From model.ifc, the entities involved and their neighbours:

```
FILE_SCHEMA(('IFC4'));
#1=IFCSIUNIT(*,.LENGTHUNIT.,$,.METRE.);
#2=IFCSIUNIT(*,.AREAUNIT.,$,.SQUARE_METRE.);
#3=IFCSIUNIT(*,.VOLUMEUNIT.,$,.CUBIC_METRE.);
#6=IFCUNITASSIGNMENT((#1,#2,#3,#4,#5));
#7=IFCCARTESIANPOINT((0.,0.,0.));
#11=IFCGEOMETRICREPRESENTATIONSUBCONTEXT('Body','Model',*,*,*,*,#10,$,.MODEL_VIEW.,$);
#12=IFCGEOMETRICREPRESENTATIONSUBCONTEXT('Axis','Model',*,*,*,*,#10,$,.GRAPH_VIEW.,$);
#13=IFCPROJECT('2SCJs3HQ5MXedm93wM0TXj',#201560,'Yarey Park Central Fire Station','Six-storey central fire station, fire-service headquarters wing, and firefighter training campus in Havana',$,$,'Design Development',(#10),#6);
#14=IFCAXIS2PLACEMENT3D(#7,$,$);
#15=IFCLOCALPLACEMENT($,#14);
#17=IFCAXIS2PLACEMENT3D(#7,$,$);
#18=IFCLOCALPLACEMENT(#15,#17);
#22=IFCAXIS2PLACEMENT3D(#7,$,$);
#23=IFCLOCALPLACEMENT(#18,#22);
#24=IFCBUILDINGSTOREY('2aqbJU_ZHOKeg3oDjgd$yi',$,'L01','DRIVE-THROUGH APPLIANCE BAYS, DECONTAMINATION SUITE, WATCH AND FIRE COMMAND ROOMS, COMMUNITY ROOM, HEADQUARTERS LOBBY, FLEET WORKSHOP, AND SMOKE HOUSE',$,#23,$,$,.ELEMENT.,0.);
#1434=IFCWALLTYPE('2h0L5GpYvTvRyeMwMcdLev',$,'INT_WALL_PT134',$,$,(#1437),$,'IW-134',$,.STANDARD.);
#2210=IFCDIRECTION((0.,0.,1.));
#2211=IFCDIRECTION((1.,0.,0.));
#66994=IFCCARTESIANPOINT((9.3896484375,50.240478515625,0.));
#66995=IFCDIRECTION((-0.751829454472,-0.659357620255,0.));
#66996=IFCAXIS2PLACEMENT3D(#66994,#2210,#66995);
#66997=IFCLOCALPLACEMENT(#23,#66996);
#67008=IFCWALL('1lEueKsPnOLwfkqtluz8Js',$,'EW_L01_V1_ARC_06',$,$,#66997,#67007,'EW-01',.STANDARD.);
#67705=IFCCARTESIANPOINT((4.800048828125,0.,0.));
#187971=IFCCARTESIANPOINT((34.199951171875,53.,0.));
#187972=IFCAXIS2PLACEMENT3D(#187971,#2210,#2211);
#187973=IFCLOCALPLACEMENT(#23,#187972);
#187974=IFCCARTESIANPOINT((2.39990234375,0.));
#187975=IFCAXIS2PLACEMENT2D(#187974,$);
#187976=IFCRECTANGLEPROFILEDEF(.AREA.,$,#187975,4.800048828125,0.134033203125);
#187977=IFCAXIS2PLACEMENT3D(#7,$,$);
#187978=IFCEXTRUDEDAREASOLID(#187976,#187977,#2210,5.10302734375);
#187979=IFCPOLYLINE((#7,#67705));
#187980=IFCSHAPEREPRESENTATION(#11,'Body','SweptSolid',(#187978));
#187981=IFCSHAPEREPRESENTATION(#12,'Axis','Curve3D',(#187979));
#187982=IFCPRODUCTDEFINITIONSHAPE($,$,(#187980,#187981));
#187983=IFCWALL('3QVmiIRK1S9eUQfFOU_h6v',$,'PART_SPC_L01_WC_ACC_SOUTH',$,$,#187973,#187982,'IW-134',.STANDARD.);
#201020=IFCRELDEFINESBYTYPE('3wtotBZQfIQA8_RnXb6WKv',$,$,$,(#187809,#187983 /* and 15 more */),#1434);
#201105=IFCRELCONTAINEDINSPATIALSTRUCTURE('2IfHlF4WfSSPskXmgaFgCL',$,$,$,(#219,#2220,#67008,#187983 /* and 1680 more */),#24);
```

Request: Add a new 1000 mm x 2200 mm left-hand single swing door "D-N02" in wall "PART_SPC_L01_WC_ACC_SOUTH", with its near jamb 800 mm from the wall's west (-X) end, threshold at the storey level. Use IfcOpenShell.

```python
import numpy as np
import ifcopenshell
import ifcopenshell.api.feature
import ifcopenshell.api.geometry
import ifcopenshell.api.root
import ifcopenshell.api.spatial
import ifcopenshell.geom
import ifcopenshell.util.element
import ifcopenshell.util.placement
import ifcopenshell.util.representation
import ifcopenshell.util.shape
import ifcopenshell.util.unit

model = ifcopenshell.open("model.ifc")
unit_scale = ifcopenshell.util.unit.calculate_unit_scale(model)
settings = ifcopenshell.geom.settings()


def volume(element):
    """Net volume in cubic metres, openings subtracted."""
    shape = ifcopenshell.geom.create_shape(settings, element)
    return ifcopenshell.util.shape.get_volume(shape.geometry)


wall = model.by_guid("3QVmiIRK1S9eUQfFOU_h6v")
storey = ifcopenshell.util.element.get_container(wall, ifc_class="IfcBuildingStorey")
context = ifcopenshell.util.representation.get_context(model, "Model", "Body", "MODEL_VIEW")
before = volume(wall)

width, height, from_end, sill = 1, 2.2, 0.8, 0.0  # metres

# The wall runs along its own X axis, and the end named is its -X end.
wall_shape = ifcopenshell.geom.create_shape(settings, wall)
x, y, z = ifcopenshell.util.shape.get_vertices(wall_shape.geometry).T
start = x.min() + from_end
face, thickness = float(y.min()), float(y.max() - y.min())
wall_matrix = ifcopenshell.util.placement.get_local_placement(wall.ObjectPlacement)
level = ifcopenshell.util.placement.get_local_placement(storey.ObjectPlacement)[2, 3]


def in_wall(x, y):
    """Placement at x, y metres in the wall's axes, at sill height."""
    matrix = wall_matrix.copy()
    matrix[:, 3] = wall_matrix @ np.array([x / unit_scale, y / unit_scale, 0.0, 1.0])
    matrix[2, 3] = level + sill / unit_scale
    return matrix


# Opening: a box that overshoots both wall faces by 50 mm.
opening = ifcopenshell.api.root.create_entity(model, ifc_class="IfcOpeningElement", predefined_type="OPENING")
box = ifcopenshell.api.geometry.add_wall_representation(
    model, context=context, length=width, height=height, thickness=thickness + 0.1
)
ifcopenshell.api.geometry.assign_representation(model, product=opening, representation=box)
ifcopenshell.api.geometry.edit_object_placement(model, product=opening, matrix=in_wall(start, face - 0.05), is_si=False)
ifcopenshell.api.feature.add_feature(model, feature=opening, element=wall)

door = ifcopenshell.api.root.create_entity(model, ifc_class="IfcDoor", name="D-N02", predefined_type="DOOR")
door.OverallWidth, door.OverallHeight = width / unit_scale, height / unit_scale
door.OperationType = "SINGLE_SWING_LEFT"
body = ifcopenshell.api.geometry.add_door_representation(
    model,
    context=context,
    overall_width=door.OverallWidth,
    overall_height=door.OverallHeight,
    operation_type="SINGLE_SWING_LEFT",
    lining_properties={"LiningDepth": thickness / unit_scale, "ThresholdDepth": thickness / unit_scale},
)
ifcopenshell.api.geometry.assign_representation(model, product=door, representation=body)
ifcopenshell.api.spatial.assign_container(model, products=[door], relating_structure=storey)
ifcopenshell.api.feature.add_filling(model, opening=opening, element=door)

# The lining spans the wall, so the door starts at the wall face.
ifcopenshell.api.geometry.edit_object_placement(model, product=door, matrix=in_wall(start, face), is_si=False)

after = volume(wall)

print(f"wall volume {before:.3f} -> {after:.3f} m3")

model.write("model_v2.ifc")
```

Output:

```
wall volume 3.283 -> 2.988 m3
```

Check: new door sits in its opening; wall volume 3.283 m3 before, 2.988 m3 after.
